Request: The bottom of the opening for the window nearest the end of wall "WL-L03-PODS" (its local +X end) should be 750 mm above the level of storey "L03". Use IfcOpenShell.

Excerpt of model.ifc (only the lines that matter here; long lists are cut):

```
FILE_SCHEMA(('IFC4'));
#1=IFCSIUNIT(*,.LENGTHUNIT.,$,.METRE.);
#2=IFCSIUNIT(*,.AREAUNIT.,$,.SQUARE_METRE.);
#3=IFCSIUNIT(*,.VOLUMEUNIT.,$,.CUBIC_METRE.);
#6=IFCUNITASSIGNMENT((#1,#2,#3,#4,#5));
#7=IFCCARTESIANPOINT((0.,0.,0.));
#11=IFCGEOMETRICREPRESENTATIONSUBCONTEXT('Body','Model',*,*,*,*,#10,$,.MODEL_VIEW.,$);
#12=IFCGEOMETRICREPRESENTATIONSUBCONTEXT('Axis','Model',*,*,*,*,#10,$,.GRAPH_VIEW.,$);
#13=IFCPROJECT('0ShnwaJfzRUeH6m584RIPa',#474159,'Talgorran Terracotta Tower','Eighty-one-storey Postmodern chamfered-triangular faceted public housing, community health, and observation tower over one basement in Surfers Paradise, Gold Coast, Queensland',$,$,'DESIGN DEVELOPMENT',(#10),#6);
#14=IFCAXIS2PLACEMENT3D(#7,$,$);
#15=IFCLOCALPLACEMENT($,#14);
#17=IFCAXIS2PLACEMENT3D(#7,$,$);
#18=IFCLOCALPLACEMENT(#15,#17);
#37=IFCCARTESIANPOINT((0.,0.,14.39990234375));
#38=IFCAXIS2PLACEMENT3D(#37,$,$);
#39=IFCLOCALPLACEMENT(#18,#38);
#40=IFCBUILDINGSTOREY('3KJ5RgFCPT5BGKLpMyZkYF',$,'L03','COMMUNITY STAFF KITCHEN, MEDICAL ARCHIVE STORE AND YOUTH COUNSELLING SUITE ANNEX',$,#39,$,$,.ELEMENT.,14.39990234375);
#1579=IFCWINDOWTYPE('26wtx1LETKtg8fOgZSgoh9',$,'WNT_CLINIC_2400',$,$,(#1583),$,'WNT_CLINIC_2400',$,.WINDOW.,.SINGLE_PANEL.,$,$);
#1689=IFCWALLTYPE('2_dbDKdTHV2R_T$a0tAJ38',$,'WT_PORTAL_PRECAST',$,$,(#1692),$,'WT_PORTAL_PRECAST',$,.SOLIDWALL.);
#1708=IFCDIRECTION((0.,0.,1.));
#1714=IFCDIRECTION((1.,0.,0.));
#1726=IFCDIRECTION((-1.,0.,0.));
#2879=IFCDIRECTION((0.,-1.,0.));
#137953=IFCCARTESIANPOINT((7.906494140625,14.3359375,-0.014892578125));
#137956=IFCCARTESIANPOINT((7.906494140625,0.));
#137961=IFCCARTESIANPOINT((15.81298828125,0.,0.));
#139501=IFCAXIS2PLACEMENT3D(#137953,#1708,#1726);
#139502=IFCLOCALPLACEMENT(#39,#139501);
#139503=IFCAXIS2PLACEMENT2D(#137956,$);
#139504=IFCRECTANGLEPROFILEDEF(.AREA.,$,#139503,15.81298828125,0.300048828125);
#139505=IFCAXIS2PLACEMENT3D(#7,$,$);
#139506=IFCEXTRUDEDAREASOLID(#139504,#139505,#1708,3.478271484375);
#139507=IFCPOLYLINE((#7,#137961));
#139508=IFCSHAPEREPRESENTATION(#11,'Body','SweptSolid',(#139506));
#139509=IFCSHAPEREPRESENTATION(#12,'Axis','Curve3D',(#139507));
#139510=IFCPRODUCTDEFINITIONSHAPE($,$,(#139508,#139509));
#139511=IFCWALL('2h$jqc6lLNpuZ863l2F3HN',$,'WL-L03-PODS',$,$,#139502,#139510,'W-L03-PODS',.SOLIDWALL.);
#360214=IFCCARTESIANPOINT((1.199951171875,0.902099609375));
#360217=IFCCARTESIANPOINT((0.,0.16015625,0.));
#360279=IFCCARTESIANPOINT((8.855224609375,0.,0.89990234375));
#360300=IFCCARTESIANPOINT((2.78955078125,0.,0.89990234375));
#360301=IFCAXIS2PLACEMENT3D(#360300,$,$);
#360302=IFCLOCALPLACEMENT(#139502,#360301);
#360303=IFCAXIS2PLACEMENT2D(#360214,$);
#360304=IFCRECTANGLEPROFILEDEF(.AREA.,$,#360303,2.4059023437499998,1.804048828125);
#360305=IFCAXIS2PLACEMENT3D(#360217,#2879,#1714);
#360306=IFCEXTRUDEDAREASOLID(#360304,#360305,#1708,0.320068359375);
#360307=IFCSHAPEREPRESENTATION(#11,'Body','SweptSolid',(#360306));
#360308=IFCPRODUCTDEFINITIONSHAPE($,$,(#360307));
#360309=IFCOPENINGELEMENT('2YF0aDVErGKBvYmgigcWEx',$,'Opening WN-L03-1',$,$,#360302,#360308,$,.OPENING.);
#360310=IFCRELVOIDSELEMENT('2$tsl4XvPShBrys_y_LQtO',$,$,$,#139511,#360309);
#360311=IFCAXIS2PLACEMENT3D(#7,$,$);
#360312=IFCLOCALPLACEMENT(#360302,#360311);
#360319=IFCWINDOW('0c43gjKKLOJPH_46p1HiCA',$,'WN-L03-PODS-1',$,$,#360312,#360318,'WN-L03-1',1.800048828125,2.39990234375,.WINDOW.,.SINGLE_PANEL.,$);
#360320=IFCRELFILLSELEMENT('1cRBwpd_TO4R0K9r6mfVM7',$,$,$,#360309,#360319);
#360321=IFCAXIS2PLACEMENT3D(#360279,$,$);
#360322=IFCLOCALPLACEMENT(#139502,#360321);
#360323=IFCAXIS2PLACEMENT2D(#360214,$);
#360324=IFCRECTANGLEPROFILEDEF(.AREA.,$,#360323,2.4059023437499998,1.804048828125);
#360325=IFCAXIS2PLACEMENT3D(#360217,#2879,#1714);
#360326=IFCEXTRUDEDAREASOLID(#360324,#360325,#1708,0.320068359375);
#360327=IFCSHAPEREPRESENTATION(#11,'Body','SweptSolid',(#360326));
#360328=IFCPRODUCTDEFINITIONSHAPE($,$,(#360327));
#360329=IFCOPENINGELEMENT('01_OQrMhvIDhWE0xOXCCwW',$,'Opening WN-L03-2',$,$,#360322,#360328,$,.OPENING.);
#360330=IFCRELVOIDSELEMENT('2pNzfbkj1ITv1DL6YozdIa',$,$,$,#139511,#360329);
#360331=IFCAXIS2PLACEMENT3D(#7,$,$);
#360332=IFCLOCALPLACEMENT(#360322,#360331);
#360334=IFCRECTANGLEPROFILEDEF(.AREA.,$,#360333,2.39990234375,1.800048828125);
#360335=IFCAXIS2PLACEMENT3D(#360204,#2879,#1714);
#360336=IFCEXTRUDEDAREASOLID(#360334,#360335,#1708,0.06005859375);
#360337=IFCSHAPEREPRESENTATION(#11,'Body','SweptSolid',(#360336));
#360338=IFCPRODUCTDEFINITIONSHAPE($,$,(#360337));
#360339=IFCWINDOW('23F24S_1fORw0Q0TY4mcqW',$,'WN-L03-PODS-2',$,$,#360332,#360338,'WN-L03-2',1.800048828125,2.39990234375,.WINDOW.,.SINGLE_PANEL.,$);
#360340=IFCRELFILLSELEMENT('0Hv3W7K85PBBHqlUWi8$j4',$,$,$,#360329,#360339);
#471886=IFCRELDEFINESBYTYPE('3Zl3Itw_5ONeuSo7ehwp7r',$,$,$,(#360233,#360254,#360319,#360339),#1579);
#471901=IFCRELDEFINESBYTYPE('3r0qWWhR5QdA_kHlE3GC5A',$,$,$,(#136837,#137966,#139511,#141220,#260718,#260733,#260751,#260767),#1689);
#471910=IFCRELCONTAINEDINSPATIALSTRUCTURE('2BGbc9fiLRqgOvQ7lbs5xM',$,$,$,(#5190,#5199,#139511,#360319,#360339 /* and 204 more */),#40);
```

```python
import numpy as np
import ifcopenshell
import ifcopenshell.api.geometry
import ifcopenshell.geom
import ifcopenshell.util.element
import ifcopenshell.util.placement
import ifcopenshell.util.shape
import ifcopenshell.util.unit

model = ifcopenshell.open("model.ifc")
unit_scale = ifcopenshell.util.unit.calculate_unit_scale(model)

window = model.by_guid("23F24S_1fORw0Q0TY4mcqW")
opening = window.FillsVoids[0].RelatingOpeningElement
storey = ifcopenshell.util.element.get_container(window, ifc_class="IfcBuildingStorey")
level = ifcopenshell.util.placement.get_local_placement(storey.ObjectPlacement)[2, 3]

# The opening's origin need not be at the sill, so measure its lowest point.
shape = ifcopenshell.geom.create_shape(ifcopenshell.geom.settings(), opening)
bottom = ifcopenshell.util.shape.get_shape_bottom_elevation(shape, shape.geometry) / unit_scale
dz = level + 0.75 - bottom

shift = np.array([0.0, 0.0, dz])
# The window is placed relative to its opening, so it follows when the opening moves.
matrix = ifcopenshell.util.placement.get_local_placement(opening.ObjectPlacement)
matrix[:3, 3] += shift
ifcopenshell.api.geometry.edit_object_placement(
    model, product=opening, matrix=matrix, is_si=False, should_transform_children=True
)

print(f"moved by {dz * unit_scale:+.3f} m")

model.write("model-out.ifc")
```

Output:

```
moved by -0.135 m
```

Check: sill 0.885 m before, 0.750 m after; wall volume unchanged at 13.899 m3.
